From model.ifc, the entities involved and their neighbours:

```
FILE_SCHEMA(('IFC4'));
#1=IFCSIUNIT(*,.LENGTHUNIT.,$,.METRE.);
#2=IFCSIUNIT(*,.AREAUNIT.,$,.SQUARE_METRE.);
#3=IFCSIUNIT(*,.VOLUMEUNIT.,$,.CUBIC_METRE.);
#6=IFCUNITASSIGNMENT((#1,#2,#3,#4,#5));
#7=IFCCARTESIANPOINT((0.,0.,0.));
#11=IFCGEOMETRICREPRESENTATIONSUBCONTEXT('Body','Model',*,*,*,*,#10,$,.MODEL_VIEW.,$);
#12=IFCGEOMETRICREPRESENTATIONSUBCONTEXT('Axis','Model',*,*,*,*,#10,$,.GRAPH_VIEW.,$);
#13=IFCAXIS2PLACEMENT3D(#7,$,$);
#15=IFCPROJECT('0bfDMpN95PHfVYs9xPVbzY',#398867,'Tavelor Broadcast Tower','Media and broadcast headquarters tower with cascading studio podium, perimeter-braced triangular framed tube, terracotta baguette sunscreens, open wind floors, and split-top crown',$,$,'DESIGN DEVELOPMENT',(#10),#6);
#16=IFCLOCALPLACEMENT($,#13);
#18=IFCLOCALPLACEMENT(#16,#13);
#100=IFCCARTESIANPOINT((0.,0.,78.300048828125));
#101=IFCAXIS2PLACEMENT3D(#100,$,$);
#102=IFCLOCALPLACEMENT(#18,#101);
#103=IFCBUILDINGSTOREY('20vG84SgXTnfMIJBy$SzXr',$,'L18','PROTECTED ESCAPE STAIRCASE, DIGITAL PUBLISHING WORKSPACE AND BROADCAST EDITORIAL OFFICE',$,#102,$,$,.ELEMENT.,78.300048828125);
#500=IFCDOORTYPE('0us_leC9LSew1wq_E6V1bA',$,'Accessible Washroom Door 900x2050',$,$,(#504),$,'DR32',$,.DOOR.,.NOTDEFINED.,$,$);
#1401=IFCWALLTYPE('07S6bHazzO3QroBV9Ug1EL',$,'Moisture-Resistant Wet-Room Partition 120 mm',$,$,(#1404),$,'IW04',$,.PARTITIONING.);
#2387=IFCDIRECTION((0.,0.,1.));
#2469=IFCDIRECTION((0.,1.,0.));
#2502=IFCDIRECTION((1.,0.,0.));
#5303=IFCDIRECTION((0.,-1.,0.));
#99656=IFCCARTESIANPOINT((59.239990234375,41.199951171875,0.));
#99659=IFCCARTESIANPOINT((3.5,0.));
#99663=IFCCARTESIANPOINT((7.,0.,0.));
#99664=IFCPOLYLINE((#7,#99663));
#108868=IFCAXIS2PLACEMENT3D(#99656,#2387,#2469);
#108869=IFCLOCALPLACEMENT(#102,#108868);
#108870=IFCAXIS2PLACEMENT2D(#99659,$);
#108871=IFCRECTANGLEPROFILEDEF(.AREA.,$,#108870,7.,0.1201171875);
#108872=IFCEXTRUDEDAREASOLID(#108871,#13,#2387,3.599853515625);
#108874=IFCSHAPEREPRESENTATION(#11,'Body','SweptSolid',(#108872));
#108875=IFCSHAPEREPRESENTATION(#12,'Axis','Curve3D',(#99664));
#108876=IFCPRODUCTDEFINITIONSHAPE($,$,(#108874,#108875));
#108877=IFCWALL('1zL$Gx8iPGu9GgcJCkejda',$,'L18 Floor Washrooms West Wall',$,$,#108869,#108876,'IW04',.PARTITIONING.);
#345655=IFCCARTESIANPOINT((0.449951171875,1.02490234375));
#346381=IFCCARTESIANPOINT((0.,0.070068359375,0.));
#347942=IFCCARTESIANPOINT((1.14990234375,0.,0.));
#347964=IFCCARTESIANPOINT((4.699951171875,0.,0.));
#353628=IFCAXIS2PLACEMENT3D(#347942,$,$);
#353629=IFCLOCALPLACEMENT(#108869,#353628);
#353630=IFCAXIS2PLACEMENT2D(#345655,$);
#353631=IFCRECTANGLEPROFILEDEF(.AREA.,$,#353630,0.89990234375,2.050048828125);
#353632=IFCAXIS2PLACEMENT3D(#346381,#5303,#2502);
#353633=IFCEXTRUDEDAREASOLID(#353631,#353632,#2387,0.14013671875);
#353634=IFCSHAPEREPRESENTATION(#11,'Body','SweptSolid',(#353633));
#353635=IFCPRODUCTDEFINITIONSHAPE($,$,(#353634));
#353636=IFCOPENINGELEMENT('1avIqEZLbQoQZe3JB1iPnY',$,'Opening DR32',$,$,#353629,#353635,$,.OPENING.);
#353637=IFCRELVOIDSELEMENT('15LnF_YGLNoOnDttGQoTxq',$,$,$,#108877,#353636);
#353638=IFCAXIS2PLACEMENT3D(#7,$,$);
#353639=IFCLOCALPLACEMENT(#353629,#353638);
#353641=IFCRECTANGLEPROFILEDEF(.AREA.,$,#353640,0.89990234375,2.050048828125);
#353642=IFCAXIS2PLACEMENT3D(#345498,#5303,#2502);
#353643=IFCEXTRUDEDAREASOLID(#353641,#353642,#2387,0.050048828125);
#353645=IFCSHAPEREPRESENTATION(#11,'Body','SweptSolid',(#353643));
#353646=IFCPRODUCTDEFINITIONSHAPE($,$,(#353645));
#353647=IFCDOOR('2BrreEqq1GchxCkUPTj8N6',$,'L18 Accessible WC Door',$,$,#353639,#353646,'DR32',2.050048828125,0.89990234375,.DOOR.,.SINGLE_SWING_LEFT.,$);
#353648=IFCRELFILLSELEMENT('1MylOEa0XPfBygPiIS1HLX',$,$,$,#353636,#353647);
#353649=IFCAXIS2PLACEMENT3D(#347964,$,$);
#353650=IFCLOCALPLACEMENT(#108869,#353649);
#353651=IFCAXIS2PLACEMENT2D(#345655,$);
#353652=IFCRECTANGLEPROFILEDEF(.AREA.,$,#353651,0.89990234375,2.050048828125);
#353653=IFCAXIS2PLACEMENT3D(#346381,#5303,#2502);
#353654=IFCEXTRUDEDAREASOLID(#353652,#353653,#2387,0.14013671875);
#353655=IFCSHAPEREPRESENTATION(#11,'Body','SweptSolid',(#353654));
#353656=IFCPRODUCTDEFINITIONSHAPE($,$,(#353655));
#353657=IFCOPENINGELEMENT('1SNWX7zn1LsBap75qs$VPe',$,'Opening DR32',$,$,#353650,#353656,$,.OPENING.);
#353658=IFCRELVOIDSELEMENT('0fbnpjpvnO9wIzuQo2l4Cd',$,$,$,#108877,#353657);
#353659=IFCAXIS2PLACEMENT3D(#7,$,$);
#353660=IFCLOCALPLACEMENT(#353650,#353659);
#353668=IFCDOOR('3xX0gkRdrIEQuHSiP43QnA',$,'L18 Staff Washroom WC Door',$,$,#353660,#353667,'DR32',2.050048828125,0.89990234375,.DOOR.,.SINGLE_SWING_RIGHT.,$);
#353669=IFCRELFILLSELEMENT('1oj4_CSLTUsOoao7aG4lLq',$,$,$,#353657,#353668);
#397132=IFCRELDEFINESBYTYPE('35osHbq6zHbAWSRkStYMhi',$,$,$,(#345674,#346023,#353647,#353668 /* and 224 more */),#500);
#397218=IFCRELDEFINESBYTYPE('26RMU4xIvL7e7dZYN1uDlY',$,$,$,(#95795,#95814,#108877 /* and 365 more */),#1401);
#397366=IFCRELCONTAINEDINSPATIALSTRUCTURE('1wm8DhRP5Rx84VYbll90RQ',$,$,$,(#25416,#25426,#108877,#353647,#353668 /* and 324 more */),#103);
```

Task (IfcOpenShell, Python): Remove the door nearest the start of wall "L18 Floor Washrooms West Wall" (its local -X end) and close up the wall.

```python
import ifcopenshell
import ifcopenshell.api.feature
import ifcopenshell.api.root
import ifcopenshell.geom
import ifcopenshell.util.shape

model = ifcopenshell.open("model.ifc")
settings = ifcopenshell.geom.settings()


def volume(element):
    """Net volume in cubic metres, openings subtracted."""
    shape = ifcopenshell.geom.create_shape(settings, element)
    return ifcopenshell.util.shape.get_volume(shape.geometry)


door = model.by_guid("2BrreEqq1GchxCkUPTj8N6")
opening = door.FillsVoids[0].RelatingOpeningElement
wall = opening.VoidsElements[0].RelatingBuildingElement
before = volume(wall)

ifcopenshell.api.root.remove_product(model, product=door)
ifcopenshell.api.feature.remove_feature(model, feature=opening)

after = volume(wall)

print(f"wall volume {before:.3f} -> {after:.3f} m3")

model.write("model_updated.ifc")
```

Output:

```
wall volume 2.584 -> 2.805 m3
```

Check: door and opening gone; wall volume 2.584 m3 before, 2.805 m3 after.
